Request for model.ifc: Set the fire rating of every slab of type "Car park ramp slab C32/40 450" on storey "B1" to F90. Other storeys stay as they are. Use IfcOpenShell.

First a look at what the model holds.

```python
import ifcopenshell
import ifcopenshell.util.element

model = ifcopenshell.open("model.ifc")
print(model.schema)
storey = next(s for s in model.by_type("IfcBuildingStorey") if s.Name == "B1")
slabs = [e for e in ifcopenshell.util.element.get_decomposition(storey) if e.is_a("IfcSlab")]
seen = {}
for e in slabs:
    element_type = ifcopenshell.util.element.get_type(e)
    key = (element_type.Name if element_type != e and element_type else None, ifcopenshell.util.element.get_pset(e, "Pset_SlabCommon", "FireRating"))
    seen[key] = seen.get(key, 0) + 1
for (name, value), count in sorted(seen.items(), key=str):
    print(count, "x", name, "|", value)
```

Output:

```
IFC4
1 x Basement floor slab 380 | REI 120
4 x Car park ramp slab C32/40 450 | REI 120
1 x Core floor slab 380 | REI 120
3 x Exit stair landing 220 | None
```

```python
import ifcopenshell
import ifcopenshell.api.pset
import ifcopenshell.util.element

model = ifcopenshell.open("model.ifc")

storey = next(s for s in model.by_type("IfcBuildingStorey") if s.Name == "B1")
slabs = [e for e in ifcopenshell.util.element.get_decomposition(storey) if e.is_a("IfcSlab")]

count = 0
for e in slabs:
    element_type = ifcopenshell.util.element.get_type(e)
    if element_type in (None, e) or element_type.Name != "Car park ramp slab C32/40 450":
        continue
    found = ifcopenshell.util.element.get_pset(e, "Pset_SlabCommon", should_inherit=False)
    if found:
        pset = model.by_id(found["id"])
        if len(ifcopenshell.util.element.get_elements_by_pset(pset)) > 1:
            pset = ifcopenshell.api.pset.unshare_pset(model, products=[e], pset=pset)[0]
    else:
        pset = ifcopenshell.api.pset.add_pset(model, product=e, name="Pset_SlabCommon")
    ifcopenshell.api.pset.edit_pset(model, pset=pset, properties={"FireRating": "F90"})
    count += 1

print(count, "slabs updated")

model.write("model_updated.ifc")
```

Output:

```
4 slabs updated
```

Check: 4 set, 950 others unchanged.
